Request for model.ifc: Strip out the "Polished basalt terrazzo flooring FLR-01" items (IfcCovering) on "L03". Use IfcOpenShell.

First a look at what the model holds.

```python
import ifcopenshell
import ifcopenshell.util.element

model = ifcopenshell.open("model.ifc")
print(model.schema)
storey = next(s for s in model.by_type("IfcBuildingStorey") if s.Name == "L03")
coverings = [e for e in ifcopenshell.util.element.get_decomposition(storey) if e.is_a("IfcCovering")]
seen = {}
for e in coverings:
    element_type = ifcopenshell.util.element.get_type(e)
    name = element_type.Name if element_type not in (None, e) else None
    seen[name] = seen.get(name, 0) + 1
for name, count in sorted(seen.items(), key=str):
    print(count, "x", name)
```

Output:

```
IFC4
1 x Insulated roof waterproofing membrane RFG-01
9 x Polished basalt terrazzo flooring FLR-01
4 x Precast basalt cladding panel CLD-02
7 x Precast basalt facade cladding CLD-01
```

```python
import ifcopenshell
import ifcopenshell.api.root
import ifcopenshell.util.element

model = ifcopenshell.open("model.ifc")

storey = next(s for s in model.by_type("IfcBuildingStorey") if s.Name == "L03")
coverings = [e for e in ifcopenshell.util.element.get_decomposition(storey) if e.is_a("IfcCovering")]
targets = [e for e in coverings if (t := ifcopenshell.util.element.get_type(e)) not in (None, e) and t.Name == "Polished basalt terrazzo flooring FLR-01"]

for e in targets:
    ifcopenshell.api.root.remove_product(model, product=e)
print(len(targets), "removed")

model.write("model_rev.ifc")
```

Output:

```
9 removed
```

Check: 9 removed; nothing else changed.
